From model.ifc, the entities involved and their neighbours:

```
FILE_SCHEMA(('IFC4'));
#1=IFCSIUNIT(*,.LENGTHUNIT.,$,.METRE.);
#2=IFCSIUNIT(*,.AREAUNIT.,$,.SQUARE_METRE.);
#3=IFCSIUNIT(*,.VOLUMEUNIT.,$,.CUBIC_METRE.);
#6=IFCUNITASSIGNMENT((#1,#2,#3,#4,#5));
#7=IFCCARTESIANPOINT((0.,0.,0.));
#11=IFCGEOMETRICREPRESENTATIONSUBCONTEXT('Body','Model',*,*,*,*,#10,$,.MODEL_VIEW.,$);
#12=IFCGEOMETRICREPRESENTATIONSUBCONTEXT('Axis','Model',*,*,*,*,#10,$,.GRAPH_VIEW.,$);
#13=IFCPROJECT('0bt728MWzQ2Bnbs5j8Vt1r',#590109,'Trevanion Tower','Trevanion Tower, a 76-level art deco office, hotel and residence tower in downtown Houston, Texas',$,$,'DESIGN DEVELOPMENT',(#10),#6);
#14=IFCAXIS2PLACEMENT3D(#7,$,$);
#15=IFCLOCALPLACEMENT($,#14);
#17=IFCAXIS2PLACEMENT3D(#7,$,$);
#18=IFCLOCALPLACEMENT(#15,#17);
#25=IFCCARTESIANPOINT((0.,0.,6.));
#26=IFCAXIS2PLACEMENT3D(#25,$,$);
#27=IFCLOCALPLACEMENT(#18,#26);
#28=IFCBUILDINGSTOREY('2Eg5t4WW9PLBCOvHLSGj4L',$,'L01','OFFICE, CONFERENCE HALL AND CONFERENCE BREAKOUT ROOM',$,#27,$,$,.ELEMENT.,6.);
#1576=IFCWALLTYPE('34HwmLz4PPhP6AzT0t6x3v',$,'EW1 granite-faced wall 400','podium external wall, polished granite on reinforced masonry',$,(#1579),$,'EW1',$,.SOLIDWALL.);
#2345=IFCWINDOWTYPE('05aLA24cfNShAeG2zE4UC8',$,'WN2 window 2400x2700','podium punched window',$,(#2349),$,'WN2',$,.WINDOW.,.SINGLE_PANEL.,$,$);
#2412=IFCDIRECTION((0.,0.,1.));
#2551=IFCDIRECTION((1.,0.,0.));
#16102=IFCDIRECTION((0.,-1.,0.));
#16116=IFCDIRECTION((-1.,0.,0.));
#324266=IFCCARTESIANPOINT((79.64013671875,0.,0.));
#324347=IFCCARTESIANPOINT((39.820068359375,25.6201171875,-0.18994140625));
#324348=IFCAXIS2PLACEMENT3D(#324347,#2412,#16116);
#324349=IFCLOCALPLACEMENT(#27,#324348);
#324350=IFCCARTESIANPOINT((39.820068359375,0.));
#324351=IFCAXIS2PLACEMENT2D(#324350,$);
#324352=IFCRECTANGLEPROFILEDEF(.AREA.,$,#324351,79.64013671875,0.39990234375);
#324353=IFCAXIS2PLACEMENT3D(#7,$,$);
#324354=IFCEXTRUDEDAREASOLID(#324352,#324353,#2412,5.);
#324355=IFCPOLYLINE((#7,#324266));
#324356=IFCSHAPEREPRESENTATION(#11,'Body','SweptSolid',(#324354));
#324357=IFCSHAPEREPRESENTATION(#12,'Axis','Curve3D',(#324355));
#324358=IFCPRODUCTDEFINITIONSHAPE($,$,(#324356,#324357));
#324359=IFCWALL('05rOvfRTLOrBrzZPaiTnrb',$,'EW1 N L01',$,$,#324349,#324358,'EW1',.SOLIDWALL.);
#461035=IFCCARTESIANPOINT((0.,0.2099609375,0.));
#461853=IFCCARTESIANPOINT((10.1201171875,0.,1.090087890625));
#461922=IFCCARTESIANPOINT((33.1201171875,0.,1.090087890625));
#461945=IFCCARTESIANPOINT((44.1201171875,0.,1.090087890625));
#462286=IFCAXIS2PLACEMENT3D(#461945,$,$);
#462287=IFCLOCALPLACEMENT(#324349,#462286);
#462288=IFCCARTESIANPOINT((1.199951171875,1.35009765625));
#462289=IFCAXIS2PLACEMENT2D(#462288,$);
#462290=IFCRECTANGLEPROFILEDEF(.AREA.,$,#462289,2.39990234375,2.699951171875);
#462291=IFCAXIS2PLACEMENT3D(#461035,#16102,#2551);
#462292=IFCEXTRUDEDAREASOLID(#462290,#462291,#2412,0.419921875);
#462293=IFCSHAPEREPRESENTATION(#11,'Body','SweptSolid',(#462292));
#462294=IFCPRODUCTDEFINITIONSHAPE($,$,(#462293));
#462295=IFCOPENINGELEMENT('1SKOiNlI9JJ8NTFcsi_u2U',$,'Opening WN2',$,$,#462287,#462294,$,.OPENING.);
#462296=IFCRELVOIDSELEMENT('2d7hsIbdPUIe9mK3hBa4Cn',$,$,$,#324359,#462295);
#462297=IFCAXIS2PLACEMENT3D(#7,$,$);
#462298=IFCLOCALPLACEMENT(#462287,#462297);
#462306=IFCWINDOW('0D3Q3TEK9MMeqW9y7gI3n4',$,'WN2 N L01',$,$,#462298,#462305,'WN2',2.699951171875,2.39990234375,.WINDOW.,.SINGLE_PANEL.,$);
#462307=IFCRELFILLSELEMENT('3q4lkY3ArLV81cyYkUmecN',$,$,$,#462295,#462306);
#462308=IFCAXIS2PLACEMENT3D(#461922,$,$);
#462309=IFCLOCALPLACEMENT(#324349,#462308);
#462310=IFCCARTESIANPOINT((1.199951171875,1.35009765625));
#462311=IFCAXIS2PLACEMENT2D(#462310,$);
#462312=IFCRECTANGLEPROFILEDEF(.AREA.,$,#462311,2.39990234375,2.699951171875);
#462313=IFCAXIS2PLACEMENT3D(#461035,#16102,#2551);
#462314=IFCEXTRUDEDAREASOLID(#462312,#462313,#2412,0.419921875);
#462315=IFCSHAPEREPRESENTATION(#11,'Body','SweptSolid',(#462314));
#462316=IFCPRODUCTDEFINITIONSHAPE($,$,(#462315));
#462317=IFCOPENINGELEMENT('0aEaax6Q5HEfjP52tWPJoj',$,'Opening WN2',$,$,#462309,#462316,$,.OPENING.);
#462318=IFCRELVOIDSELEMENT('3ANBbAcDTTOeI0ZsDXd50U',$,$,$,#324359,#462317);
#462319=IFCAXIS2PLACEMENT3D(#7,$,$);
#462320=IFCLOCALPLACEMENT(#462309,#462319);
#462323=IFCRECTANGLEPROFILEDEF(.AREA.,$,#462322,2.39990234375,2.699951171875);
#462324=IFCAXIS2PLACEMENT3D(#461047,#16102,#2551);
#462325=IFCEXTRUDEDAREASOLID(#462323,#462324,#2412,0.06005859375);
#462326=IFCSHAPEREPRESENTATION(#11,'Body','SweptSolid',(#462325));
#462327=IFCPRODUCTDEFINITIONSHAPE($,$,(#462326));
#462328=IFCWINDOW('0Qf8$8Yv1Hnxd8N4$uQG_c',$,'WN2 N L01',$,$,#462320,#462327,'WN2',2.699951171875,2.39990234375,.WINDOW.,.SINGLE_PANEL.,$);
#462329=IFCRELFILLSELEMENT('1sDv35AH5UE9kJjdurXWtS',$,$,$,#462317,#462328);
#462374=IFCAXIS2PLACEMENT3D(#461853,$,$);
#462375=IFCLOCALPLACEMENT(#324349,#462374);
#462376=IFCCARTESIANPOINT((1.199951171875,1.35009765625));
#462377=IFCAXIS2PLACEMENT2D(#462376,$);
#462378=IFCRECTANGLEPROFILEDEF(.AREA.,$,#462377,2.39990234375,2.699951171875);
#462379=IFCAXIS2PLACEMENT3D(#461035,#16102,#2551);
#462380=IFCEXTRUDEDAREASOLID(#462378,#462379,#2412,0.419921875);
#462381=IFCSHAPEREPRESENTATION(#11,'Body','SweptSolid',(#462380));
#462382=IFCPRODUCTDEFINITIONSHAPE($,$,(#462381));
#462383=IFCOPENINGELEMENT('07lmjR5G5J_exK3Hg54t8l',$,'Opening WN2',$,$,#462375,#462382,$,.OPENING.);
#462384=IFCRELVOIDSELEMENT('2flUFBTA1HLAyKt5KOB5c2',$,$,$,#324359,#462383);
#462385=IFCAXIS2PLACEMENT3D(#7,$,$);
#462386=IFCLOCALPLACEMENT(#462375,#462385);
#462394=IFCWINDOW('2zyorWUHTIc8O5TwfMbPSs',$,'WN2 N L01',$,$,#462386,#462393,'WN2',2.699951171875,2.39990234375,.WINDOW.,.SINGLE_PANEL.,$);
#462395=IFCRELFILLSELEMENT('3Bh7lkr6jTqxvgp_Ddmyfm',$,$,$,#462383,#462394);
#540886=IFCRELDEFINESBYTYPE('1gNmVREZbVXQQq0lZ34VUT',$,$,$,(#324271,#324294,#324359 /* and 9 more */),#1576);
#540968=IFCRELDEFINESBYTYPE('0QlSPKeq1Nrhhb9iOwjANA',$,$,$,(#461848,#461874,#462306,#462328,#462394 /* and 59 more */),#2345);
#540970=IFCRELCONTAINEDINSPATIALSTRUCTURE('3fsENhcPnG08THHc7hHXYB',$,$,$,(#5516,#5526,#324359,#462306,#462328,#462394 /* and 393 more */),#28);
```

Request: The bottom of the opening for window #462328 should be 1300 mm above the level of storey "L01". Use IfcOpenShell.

```python
import numpy as np
import ifcopenshell
import ifcopenshell.api.geometry
import ifcopenshell.geom
import ifcopenshell.util.element
import ifcopenshell.util.placement
import ifcopenshell.util.shape
import ifcopenshell.util.unit

model = ifcopenshell.open("model.ifc")
unit_scale = ifcopenshell.util.unit.calculate_unit_scale(model)

window = model.by_guid("0Qf8$8Yv1Hnxd8N4$uQG_c")
opening = window.FillsVoids[0].RelatingOpeningElement
storey = ifcopenshell.util.element.get_container(window, ifc_class="IfcBuildingStorey")
level = ifcopenshell.util.placement.get_local_placement(storey.ObjectPlacement)[2, 3]

# The opening's origin need not be at the sill, so measure its lowest point.
shape = ifcopenshell.geom.create_shape(ifcopenshell.geom.settings(), opening)
bottom = ifcopenshell.util.shape.get_shape_bottom_elevation(shape, shape.geometry) / unit_scale
dz = level + 1.3 - bottom

shift = np.array([0.0, 0.0, dz])
# The window is placed relative to its opening, so it follows when the opening moves.
matrix = ifcopenshell.util.placement.get_local_placement(opening.ObjectPlacement)
matrix[:3, 3] += shift
ifcopenshell.api.geometry.edit_object_placement(
    model, product=opening, matrix=matrix, is_si=False, should_transform_children=True
)

print(f"moved by {dz * unit_scale:+.3f} m")

model.write("model_edited.ifc")
```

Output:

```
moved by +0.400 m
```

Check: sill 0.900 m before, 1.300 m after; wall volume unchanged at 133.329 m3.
